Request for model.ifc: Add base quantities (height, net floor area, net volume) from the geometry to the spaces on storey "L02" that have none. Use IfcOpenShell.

First a look at what the model holds.

```python
import ifcopenshell
import ifcopenshell.util.element
import ifcopenshell.util.unit

model = ifcopenshell.open("model.ifc")
print(model.schema)
for unit_type in ("LENGTHUNIT", "AREAUNIT", "VOLUMEUNIT"):
    print(unit_type, ifcopenshell.util.unit.calculate_unit_scale(model, unit_type))
storey = next(s for s in model.by_type("IfcBuildingStorey") if s.Name == "L02")
spaces = [e for e in ifcopenshell.util.element.get_decomposition(storey) if e.is_a("IfcSpace")]
for e in sorted(spaces, key=lambda e: e.id()):
    print(e.id(), e.is_a(), e.Name, list(ifcopenshell.util.element.get_psets(e, qtos_only=True)), sep=" | ")
```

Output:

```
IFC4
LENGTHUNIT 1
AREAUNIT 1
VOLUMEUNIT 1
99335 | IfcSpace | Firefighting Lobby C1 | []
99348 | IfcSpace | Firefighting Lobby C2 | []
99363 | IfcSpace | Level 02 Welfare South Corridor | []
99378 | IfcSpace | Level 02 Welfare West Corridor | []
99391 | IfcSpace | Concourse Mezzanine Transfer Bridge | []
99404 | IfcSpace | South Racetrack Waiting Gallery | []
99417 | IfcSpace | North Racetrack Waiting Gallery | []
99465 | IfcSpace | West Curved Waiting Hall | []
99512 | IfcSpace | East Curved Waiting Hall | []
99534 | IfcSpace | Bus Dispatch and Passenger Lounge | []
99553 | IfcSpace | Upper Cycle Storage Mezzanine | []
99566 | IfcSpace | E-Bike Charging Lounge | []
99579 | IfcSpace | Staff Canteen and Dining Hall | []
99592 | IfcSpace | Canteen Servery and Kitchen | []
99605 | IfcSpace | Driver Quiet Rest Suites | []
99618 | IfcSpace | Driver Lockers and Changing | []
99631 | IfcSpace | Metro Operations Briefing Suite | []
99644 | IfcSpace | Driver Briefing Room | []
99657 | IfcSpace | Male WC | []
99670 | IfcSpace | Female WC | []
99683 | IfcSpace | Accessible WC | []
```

```python
import ifcopenshell
import ifcopenshell.api.pset
import ifcopenshell.geom
import ifcopenshell.util.element
import ifcopenshell.util.shape
import ifcopenshell.util.unit

model = ifcopenshell.open("model.ifc")
unit_scale = ifcopenshell.util.unit.calculate_unit_scale(model)
area_scale = ifcopenshell.util.unit.calculate_unit_scale(model, "AREAUNIT")
volume_scale = ifcopenshell.util.unit.calculate_unit_scale(model, "VOLUMEUNIT")
settings = ifcopenshell.geom.settings()

storey = next(s for s in model.by_type("IfcBuildingStorey") if s.Name == "L02")
spaces = [e for e in ifcopenshell.util.element.get_decomposition(storey) if e.is_a("IfcSpace")]

for e in sorted(spaces, key=lambda e: e.id()):
    if ifcopenshell.util.element.get_psets(e, qtos_only=True, should_inherit=False):
        continue
    # Geometry comes back in metres, in the element's own axes.
    shape = ifcopenshell.geom.create_shape(settings, e)
    values = {
        "Height": ifcopenshell.util.shape.get_z(shape.geometry) / unit_scale,
        "NetFloorArea": ifcopenshell.util.shape.get_footprint_area(shape.geometry) / area_scale,
        "NetVolume": ifcopenshell.util.shape.get_volume(shape.geometry) / volume_scale,
    }
    qto = ifcopenshell.api.pset.add_qto(model, product=e, name="Qto_SpaceBaseQuantities")
    ifcopenshell.api.pset.edit_qto(model, qto=qto, properties=values)
    print(e.id(), {k: round(v, 3) for k, v in values.items()})

model.write("model_v2.ifc")
```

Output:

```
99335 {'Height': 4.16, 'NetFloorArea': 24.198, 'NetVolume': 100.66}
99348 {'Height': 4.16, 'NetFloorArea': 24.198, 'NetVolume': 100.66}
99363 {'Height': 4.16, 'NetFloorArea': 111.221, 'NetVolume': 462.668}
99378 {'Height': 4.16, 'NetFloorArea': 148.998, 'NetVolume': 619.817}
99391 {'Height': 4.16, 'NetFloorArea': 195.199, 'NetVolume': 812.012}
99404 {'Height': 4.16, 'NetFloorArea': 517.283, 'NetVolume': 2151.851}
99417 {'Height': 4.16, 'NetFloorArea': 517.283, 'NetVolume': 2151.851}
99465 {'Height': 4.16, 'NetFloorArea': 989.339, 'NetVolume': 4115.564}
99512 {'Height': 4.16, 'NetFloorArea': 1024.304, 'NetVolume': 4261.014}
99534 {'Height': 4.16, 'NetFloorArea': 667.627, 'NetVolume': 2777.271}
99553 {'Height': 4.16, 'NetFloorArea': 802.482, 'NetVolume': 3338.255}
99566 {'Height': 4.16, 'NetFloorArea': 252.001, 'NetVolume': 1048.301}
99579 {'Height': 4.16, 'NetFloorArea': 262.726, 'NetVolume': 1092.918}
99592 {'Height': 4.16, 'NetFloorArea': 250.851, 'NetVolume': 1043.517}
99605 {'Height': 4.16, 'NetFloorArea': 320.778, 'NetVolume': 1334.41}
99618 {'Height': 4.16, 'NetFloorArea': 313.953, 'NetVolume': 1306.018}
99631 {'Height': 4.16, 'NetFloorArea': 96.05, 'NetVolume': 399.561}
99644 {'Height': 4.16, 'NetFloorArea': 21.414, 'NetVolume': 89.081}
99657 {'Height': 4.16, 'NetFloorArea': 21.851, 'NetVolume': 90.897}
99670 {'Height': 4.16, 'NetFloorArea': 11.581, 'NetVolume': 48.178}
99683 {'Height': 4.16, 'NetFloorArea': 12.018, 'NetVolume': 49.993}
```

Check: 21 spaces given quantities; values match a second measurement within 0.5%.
